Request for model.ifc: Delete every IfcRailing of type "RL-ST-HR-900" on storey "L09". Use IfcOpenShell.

First a look at what the model holds.

```python
import ifcopenshell
import ifcopenshell.util.element

model = ifcopenshell.open("model.ifc")
print(model.schema)
storey = next(s for s in model.by_type("IfcBuildingStorey") if s.Name == "L09")
railings = [e for e in ifcopenshell.util.element.get_decomposition(storey) if e.is_a("IfcRailing")]
seen = {}
for e in railings:
    element_type = ifcopenshell.util.element.get_type(e)
    name = element_type.Name if element_type not in (None, e) else None
    seen[name] = seen.get(name, 0) + 1
for name, count in sorted(seen.items(), key=str):
    print(count, "x", name)
```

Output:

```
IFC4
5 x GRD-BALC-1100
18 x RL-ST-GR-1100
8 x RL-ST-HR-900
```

```python
import ifcopenshell
import ifcopenshell.api.root
import ifcopenshell.util.element

model = ifcopenshell.open("model.ifc")

storey = next(s for s in model.by_type("IfcBuildingStorey") if s.Name == "L09")
railings = [e for e in ifcopenshell.util.element.get_decomposition(storey) if e.is_a("IfcRailing")]
targets = [e for e in railings if (t := ifcopenshell.util.element.get_type(e)) not in (None, e) and t.Name == "RL-ST-HR-900"]

for e in targets:
    ifcopenshell.api.root.remove_product(model, product=e)
print(len(targets), "removed")

model.write("model_rev.ifc")
```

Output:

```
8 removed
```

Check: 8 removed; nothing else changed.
